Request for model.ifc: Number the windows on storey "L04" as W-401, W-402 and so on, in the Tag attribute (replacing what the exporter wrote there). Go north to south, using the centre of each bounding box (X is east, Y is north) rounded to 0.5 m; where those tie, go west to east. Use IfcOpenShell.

First a look at what the model holds.

```python
import ifcopenshell
import ifcopenshell.util.element
import ifcopenshell.util.placement

model = ifcopenshell.open("model.ifc")
print(model.schema)
storey = next(s for s in model.by_type("IfcBuildingStorey") if s.Name == "L04")
windows = [e for e in ifcopenshell.util.element.get_decomposition(storey) if e.is_a("IfcWindow")]
for e in sorted(windows, key=lambda e: e.id()):
    origin = ifcopenshell.util.placement.get_local_placement(e.ObjectPlacement)[:3, 3]
    print(e.id(), e.Tag, e.Name, origin.round(2) + 0.0, sep=" | ")
```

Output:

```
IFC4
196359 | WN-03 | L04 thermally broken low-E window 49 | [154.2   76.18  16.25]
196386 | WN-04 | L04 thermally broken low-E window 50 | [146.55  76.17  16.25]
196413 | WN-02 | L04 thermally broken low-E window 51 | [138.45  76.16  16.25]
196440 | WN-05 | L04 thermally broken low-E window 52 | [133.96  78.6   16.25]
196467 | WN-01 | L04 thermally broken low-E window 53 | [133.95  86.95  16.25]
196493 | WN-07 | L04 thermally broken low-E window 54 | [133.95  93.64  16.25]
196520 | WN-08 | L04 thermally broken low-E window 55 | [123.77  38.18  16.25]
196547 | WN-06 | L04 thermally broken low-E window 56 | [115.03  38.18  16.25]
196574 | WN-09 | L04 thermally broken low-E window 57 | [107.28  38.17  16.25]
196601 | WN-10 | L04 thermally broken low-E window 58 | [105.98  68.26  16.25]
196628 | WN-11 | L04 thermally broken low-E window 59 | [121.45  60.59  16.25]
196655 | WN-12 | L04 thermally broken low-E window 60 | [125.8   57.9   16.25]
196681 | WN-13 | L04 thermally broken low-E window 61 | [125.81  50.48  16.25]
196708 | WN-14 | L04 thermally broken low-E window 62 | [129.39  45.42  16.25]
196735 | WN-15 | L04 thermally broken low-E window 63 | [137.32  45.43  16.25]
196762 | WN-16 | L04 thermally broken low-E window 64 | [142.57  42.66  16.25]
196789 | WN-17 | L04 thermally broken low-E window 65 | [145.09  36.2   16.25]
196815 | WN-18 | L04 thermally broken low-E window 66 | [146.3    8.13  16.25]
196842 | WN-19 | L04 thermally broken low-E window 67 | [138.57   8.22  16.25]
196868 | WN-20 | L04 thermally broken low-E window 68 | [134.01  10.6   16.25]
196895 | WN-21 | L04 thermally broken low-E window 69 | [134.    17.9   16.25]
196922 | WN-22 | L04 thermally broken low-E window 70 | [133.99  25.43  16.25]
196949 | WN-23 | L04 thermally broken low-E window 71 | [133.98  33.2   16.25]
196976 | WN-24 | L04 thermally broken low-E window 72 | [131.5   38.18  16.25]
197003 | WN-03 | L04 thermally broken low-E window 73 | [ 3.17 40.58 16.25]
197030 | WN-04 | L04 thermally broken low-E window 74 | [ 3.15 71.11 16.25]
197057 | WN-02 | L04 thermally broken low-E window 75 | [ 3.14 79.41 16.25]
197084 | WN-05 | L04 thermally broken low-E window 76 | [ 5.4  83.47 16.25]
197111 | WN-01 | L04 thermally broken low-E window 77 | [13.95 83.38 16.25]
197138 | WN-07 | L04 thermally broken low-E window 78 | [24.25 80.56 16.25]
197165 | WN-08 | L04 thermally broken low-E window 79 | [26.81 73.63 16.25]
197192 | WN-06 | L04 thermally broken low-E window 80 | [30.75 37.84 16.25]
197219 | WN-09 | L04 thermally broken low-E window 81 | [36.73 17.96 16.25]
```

```python
import ifcopenshell
import ifcopenshell.geom
import ifcopenshell.util.element
import ifcopenshell.util.shape

model = ifcopenshell.open("model.ifc")
settings = ifcopenshell.geom.settings()
settings.set("use-world-coords", True)


def centre(element):
    shape = ifcopenshell.geom.create_shape(settings, element)
    return ifcopenshell.util.shape.get_bbox_centroid(shape.geometry)


storey = next(s for s in model.by_type("IfcBuildingStorey") if s.Name == "L04")
windows = [e for e in ifcopenshell.util.element.get_decomposition(storey) if e.is_a("IfcWindow")]

# Insertion points can sit at a corner or the storey origin, so sort by the geometry (in metres).
centres = {e: centre(e) for e in windows}
windows.sort(key=lambda e: (-round(centres[e][1] / 0.5), centres[e][0]))

for i, e in enumerate(windows, start=1):
    number = f"W-4{i:02d}"
    e.Tag = number
    print(e.id(), number)

model.write("model_edited.ifc")
```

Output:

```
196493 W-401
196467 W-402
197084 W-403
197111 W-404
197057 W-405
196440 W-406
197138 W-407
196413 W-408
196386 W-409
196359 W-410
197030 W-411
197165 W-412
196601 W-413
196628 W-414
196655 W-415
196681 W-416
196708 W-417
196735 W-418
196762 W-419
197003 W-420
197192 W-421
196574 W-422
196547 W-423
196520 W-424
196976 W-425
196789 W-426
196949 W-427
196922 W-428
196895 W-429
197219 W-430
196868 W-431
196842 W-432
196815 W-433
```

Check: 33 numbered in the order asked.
